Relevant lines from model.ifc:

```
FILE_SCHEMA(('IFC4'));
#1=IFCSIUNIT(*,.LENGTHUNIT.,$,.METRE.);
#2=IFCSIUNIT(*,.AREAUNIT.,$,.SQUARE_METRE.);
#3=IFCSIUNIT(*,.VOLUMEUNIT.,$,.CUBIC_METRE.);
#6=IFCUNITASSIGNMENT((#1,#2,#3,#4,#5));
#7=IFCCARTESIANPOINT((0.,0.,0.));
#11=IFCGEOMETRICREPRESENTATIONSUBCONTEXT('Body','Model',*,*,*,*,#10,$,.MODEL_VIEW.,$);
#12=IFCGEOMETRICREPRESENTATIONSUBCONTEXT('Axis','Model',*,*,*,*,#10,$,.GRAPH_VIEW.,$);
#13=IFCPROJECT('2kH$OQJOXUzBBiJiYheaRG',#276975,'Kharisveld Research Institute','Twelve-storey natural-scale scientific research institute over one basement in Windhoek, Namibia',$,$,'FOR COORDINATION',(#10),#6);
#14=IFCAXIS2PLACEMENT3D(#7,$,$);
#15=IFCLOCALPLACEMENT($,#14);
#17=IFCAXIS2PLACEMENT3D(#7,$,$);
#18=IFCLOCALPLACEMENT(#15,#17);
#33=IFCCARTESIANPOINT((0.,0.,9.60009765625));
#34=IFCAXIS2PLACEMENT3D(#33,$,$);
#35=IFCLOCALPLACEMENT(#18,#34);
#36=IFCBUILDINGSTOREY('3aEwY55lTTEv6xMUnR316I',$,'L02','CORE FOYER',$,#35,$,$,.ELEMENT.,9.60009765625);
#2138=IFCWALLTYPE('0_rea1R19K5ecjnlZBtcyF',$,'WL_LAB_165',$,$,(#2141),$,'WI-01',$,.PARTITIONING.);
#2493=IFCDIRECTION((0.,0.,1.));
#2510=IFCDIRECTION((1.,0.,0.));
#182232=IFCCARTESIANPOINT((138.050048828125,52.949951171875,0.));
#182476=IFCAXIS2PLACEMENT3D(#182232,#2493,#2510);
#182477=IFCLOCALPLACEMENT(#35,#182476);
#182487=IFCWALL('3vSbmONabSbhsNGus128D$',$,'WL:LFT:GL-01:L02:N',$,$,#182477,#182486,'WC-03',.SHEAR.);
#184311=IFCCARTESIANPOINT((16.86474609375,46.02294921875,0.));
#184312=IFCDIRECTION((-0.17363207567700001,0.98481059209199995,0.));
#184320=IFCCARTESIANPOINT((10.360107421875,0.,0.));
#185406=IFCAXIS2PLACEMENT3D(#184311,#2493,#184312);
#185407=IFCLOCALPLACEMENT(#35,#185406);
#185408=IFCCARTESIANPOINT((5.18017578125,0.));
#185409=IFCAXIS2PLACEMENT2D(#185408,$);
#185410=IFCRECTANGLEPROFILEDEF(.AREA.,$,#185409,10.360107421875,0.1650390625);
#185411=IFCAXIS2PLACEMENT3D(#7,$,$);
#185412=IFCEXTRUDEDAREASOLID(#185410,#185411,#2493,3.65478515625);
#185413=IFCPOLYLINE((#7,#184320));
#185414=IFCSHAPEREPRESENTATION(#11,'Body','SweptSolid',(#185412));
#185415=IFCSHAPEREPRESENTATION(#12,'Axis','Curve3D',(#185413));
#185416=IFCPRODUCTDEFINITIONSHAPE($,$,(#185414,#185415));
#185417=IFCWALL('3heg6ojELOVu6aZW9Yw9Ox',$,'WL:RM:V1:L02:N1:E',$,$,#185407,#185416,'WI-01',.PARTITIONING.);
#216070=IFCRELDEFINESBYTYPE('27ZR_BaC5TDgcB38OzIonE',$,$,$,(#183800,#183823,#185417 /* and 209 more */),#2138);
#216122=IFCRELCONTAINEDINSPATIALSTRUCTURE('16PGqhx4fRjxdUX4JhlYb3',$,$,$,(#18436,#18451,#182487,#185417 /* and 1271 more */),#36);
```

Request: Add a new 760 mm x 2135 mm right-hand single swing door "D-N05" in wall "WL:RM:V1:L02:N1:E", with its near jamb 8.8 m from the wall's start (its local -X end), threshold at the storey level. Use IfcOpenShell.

```python
import numpy as np
import ifcopenshell
import ifcopenshell.api.feature
import ifcopenshell.api.geometry
import ifcopenshell.api.root
import ifcopenshell.api.spatial
import ifcopenshell.geom
import ifcopenshell.util.element
import ifcopenshell.util.placement
import ifcopenshell.util.representation
import ifcopenshell.util.shape
import ifcopenshell.util.unit

model = ifcopenshell.open("model.ifc")
unit_scale = ifcopenshell.util.unit.calculate_unit_scale(model)
settings = ifcopenshell.geom.settings()


def volume(element):
    """Net volume in cubic metres, openings subtracted."""
    shape = ifcopenshell.geom.create_shape(settings, element)
    return ifcopenshell.util.shape.get_volume(shape.geometry)


wall = model.by_guid("3heg6ojELOVu6aZW9Yw9Ox")
storey = ifcopenshell.util.element.get_container(wall, ifc_class="IfcBuildingStorey")
context = ifcopenshell.util.representation.get_context(model, "Model", "Body", "MODEL_VIEW")
before = volume(wall)

width, height, from_end, sill = 0.76, 2.135, 8.8, 0.0  # metres

# The wall runs along its own X axis, and the end named is its -X end.
wall_shape = ifcopenshell.geom.create_shape(settings, wall)
x, y, z = ifcopenshell.util.shape.get_vertices(wall_shape.geometry).T
start = x.min() + from_end
face, thickness = float(y.min()), float(y.max() - y.min())
wall_matrix = ifcopenshell.util.placement.get_local_placement(wall.ObjectPlacement)
level = ifcopenshell.util.placement.get_local_placement(storey.ObjectPlacement)[2, 3]


def in_wall(x, y):
    """Placement at x, y metres in the wall's axes, at sill height."""
    matrix = wall_matrix.copy()
    matrix[:, 3] = wall_matrix @ np.array([x / unit_scale, y / unit_scale, 0.0, 1.0])
    matrix[2, 3] = level + sill / unit_scale
    return matrix


# Opening: a box that overshoots both wall faces by 50 mm.
opening = ifcopenshell.api.root.create_entity(model, ifc_class="IfcOpeningElement", predefined_type="OPENING")
box = ifcopenshell.api.geometry.add_wall_representation(
    model, context=context, length=width, height=height, thickness=thickness + 0.1
)
ifcopenshell.api.geometry.assign_representation(model, product=opening, representation=box)
ifcopenshell.api.geometry.edit_object_placement(model, product=opening, matrix=in_wall(start, face - 0.05), is_si=False)
ifcopenshell.api.feature.add_feature(model, feature=opening, element=wall)

door = ifcopenshell.api.root.create_entity(model, ifc_class="IfcDoor", name="D-N05", predefined_type="DOOR")
door.OverallWidth, door.OverallHeight = width / unit_scale, height / unit_scale
door.OperationType = "SINGLE_SWING_RIGHT"
body = ifcopenshell.api.geometry.add_door_representation(
    model,
    context=context,
    overall_width=door.OverallWidth,
    overall_height=door.OverallHeight,
    operation_type="SINGLE_SWING_RIGHT",
    lining_properties={"LiningDepth": thickness / unit_scale, "ThresholdDepth": thickness / unit_scale},
)
ifcopenshell.api.geometry.assign_representation(model, product=door, representation=body)
ifcopenshell.api.spatial.assign_container(model, products=[door], relating_structure=storey)
ifcopenshell.api.feature.add_filling(model, opening=opening, element=door)

# The lining spans the wall, so the door starts at the wall face.
ifcopenshell.api.geometry.edit_object_placement(model, product=door, matrix=in_wall(start, face), is_si=False)

after = volume(wall)

print(f"wall volume {before:.3f} -> {after:.3f} m3")

model.write("model_v2.ifc")
```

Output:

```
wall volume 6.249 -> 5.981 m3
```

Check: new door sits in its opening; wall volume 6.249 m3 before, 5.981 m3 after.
